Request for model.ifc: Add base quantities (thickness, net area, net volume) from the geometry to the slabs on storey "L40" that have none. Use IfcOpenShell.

First a look at what the model holds.

```python
import ifcopenshell
import ifcopenshell.util.element
import ifcopenshell.util.unit

model = ifcopenshell.open("model.ifc")
print(model.schema)
for unit_type in ("LENGTHUNIT", "AREAUNIT", "VOLUMEUNIT"):
    print(unit_type, ifcopenshell.util.unit.calculate_unit_scale(model, unit_type))
storey = next(s for s in model.by_type("IfcBuildingStorey") if s.Name == "L40")
slabs = [e for e in ifcopenshell.util.element.get_decomposition(storey) if e.is_a("IfcSlab")]
for e in sorted(slabs, key=lambda e: e.id()):
    print(e.id(), e.is_a(), e.Name, list(ifcopenshell.util.element.get_psets(e, qtos_only=True)), sep=" | ")
```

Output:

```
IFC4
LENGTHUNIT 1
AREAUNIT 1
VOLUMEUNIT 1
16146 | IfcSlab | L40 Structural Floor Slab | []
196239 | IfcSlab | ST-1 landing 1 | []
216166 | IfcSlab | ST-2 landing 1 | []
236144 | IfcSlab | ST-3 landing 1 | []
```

```python
import ifcopenshell
import ifcopenshell.api.pset
import ifcopenshell.geom
import ifcopenshell.util.element
import ifcopenshell.util.shape
import ifcopenshell.util.unit

model = ifcopenshell.open("model.ifc")
unit_scale = ifcopenshell.util.unit.calculate_unit_scale(model)
area_scale = ifcopenshell.util.unit.calculate_unit_scale(model, "AREAUNIT")
volume_scale = ifcopenshell.util.unit.calculate_unit_scale(model, "VOLUMEUNIT")
settings = ifcopenshell.geom.settings()

storey = next(s for s in model.by_type("IfcBuildingStorey") if s.Name == "L40")
slabs = [e for e in ifcopenshell.util.element.get_decomposition(storey) if e.is_a("IfcSlab")]

for e in sorted(slabs, key=lambda e: e.id()):
    if ifcopenshell.util.element.get_psets(e, qtos_only=True, should_inherit=False):
        continue
    # Geometry comes back in metres, in the element's own axes.
    shape = ifcopenshell.geom.create_shape(settings, e)
    values = {
        "Width": ifcopenshell.util.shape.get_z(shape.geometry) / unit_scale,
        "NetArea": ifcopenshell.util.shape.get_footprint_area(shape.geometry) / area_scale,
        "NetVolume": ifcopenshell.util.shape.get_volume(shape.geometry) / volume_scale,
    }
    qto = ifcopenshell.api.pset.add_qto(model, product=e, name="Qto_SlabBaseQuantities")
    ifcopenshell.api.pset.edit_qto(model, qto=qto, properties=values)
    print(e.id(), {k: round(v, 3) for k, v in values.items()})

model.write("model_rev.ifc")
```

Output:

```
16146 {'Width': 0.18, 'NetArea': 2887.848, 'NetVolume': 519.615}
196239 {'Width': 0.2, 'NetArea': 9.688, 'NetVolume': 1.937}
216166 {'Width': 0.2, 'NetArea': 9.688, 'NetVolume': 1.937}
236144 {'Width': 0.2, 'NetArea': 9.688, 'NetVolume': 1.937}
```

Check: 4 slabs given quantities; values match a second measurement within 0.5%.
